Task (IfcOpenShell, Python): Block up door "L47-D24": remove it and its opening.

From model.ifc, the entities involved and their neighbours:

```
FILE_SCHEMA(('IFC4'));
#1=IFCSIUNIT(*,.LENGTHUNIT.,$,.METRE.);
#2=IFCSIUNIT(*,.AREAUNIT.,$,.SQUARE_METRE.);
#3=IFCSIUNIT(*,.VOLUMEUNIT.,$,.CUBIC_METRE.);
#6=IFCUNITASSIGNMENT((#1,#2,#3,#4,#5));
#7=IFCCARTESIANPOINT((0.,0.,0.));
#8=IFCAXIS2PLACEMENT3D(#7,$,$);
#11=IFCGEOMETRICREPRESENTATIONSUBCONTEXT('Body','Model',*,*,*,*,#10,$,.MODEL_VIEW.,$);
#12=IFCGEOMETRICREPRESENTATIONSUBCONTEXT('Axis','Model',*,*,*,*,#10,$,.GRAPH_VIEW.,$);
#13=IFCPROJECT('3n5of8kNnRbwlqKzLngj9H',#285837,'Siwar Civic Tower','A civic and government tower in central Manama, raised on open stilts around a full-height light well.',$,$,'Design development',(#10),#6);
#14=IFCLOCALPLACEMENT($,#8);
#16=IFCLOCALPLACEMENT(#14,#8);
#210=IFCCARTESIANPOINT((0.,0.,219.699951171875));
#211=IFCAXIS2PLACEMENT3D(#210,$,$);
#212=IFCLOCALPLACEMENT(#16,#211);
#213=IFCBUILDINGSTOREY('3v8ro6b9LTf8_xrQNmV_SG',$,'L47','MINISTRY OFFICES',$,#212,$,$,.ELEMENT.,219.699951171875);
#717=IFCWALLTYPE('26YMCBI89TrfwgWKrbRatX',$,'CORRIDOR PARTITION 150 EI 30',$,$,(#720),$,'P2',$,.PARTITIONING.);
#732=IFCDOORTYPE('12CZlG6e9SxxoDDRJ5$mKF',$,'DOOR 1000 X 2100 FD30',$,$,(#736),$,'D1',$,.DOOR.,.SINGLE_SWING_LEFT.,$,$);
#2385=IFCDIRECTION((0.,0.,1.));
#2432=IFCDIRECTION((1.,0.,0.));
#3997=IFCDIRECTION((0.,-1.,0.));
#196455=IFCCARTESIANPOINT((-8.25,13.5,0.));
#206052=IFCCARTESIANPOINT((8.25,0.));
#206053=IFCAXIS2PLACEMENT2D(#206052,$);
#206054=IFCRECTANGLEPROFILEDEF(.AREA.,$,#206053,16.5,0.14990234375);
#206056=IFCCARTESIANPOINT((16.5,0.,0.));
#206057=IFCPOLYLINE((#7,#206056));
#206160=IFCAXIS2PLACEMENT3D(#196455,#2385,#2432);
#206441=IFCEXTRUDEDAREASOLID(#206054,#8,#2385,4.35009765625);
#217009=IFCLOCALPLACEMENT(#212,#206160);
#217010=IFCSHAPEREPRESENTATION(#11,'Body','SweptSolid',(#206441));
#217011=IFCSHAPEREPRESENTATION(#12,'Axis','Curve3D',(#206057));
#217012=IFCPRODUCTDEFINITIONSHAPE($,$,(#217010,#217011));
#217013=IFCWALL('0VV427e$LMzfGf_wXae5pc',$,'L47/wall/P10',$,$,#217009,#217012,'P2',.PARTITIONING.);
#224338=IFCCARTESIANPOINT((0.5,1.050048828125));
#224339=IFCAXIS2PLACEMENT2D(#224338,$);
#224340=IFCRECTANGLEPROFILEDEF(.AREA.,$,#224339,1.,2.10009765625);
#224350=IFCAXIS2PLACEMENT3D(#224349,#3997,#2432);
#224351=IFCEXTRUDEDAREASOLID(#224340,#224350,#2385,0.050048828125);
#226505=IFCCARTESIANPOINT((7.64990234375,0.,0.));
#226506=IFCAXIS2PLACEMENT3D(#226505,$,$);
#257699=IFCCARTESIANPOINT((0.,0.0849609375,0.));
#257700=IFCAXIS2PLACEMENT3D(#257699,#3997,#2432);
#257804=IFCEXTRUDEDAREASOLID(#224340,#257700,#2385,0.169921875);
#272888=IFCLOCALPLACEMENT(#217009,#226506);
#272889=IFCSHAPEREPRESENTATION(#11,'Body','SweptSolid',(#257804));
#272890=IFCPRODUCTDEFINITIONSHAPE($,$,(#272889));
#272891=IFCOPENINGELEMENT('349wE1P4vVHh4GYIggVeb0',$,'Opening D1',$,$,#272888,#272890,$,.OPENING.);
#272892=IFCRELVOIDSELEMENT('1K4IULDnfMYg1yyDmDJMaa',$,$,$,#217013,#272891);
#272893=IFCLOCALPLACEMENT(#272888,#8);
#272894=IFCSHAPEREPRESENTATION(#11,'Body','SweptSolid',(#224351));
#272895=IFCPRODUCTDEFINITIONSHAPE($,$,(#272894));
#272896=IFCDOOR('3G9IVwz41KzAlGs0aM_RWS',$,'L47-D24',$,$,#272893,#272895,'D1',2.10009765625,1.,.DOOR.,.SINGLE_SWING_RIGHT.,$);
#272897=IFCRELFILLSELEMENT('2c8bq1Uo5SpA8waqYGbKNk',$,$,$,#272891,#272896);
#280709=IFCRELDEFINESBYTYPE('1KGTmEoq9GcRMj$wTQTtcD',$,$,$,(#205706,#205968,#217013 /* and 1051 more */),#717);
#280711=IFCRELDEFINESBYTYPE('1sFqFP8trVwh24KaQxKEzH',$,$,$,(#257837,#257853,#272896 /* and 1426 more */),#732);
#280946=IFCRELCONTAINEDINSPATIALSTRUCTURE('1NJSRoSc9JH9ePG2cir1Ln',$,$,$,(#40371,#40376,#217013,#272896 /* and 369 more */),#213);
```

```python
import ifcopenshell
import ifcopenshell.api.feature
import ifcopenshell.api.root
import ifcopenshell.geom
import ifcopenshell.util.shape

model = ifcopenshell.open("model.ifc")
settings = ifcopenshell.geom.settings()


def volume(element):
    """Net volume in cubic metres, openings subtracted."""
    shape = ifcopenshell.geom.create_shape(settings, element)
    return ifcopenshell.util.shape.get_volume(shape.geometry)


door = model.by_guid("3G9IVwz41KzAlGs0aM_RWS")
opening = door.FillsVoids[0].RelatingOpeningElement
wall = opening.VoidsElements[0].RelatingBuildingElement
before = volume(wall)

ifcopenshell.api.root.remove_product(model, product=door)
ifcopenshell.api.feature.remove_feature(model, feature=opening)

after = volume(wall)

print(f"wall volume {before:.3f} -> {after:.3f} m3")

model.write("model_rev.ifc")
```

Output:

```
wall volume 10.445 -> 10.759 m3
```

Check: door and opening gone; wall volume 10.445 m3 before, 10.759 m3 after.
